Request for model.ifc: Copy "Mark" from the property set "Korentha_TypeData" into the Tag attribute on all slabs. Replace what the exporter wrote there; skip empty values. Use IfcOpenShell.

First a look at what the model holds.

```python
import ifcopenshell
import ifcopenshell.util.element

model = ifcopenshell.open("model.ifc")
print(model.schema)
slabs = model.by_type("IfcSlab")
print(len(slabs), "slabs")
for e in slabs[:8]:
    source = ifcopenshell.util.element.get_pset(e, "Korentha_TypeData", "Mark")
    target = e.Tag
    print(e.id(), repr(source), repr(target), sep=" | ")
```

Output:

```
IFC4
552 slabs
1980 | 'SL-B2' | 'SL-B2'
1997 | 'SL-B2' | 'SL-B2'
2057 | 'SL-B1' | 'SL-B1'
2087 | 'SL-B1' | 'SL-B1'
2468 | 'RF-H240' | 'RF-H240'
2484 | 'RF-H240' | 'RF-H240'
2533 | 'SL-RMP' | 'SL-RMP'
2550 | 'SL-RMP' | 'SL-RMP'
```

```python
import ifcopenshell
import ifcopenshell.util.element

model = ifcopenshell.open("model.ifc")

count = 0
for e in model.by_type("IfcSlab"):
    value = ifcopenshell.util.element.get_pset(e, "Korentha_TypeData", "Mark")
    current = e.Tag
    if not value or not value.strip() or current == value:
        continue
    e.Tag = value
    count += 1

print(count, "slabs updated")

model.write("model_v2.ifc")
```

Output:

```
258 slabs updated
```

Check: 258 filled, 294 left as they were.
